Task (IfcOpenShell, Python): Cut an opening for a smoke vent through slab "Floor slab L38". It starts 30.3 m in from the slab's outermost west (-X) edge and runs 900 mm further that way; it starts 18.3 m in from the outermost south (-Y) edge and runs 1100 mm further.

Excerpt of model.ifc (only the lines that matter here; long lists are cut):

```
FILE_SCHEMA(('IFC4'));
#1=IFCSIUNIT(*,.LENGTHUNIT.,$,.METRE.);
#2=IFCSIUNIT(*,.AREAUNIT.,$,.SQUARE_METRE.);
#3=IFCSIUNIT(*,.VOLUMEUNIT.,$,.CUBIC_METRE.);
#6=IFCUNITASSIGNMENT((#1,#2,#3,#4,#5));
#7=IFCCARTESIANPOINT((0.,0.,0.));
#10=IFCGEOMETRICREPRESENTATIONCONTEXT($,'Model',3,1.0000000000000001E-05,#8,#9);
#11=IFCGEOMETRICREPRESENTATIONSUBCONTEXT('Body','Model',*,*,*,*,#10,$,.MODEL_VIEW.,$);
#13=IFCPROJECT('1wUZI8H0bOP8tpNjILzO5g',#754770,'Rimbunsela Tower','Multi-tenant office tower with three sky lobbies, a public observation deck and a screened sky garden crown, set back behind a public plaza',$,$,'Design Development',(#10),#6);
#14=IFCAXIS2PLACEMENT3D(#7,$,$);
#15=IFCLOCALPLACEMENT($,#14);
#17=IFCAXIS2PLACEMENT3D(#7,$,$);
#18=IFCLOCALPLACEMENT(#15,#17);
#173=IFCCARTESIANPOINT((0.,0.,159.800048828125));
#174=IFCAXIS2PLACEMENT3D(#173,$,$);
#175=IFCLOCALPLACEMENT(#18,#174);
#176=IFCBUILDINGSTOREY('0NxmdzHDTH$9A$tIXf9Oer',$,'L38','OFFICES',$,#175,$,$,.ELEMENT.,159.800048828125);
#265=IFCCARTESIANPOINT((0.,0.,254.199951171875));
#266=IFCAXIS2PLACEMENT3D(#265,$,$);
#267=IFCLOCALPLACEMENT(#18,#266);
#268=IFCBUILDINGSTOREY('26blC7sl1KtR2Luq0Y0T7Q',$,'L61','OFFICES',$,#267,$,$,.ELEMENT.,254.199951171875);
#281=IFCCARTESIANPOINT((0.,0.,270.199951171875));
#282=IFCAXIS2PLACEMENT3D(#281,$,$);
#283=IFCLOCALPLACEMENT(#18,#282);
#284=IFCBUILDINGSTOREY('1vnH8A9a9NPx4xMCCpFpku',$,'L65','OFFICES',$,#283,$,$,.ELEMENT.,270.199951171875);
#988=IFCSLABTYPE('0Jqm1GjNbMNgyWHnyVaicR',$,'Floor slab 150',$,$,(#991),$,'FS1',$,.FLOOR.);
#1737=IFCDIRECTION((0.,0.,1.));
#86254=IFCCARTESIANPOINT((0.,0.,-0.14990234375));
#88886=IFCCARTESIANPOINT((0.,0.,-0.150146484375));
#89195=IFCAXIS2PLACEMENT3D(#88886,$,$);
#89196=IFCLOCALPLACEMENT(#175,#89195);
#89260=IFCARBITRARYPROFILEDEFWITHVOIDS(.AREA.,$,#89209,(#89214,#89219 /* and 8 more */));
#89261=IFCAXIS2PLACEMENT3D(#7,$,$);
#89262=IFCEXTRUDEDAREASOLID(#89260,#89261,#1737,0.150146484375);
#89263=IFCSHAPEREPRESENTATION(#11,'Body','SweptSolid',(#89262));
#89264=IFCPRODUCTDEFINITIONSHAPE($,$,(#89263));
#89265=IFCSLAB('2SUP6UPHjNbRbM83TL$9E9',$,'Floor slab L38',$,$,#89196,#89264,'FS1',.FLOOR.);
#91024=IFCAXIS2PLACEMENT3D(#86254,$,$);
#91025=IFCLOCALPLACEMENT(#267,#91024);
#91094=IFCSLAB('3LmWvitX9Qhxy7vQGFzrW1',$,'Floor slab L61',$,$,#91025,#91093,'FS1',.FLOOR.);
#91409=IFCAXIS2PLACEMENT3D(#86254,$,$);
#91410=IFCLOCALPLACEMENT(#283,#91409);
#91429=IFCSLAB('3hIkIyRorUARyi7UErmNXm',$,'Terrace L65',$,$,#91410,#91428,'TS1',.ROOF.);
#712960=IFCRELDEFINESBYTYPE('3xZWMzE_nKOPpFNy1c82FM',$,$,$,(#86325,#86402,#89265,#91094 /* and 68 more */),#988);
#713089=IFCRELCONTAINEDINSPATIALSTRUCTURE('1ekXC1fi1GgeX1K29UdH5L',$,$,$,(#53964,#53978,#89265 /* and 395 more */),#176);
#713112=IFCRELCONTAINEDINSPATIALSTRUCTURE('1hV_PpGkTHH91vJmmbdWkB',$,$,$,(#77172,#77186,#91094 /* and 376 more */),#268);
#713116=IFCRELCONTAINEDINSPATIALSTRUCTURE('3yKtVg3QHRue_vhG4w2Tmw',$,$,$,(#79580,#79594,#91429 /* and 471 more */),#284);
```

```python
import numpy as np
import ifcopenshell
import ifcopenshell.api.feature
import ifcopenshell.api.geometry
import ifcopenshell.api.root
import ifcopenshell.geom
import ifcopenshell.util.placement
import ifcopenshell.util.representation
import ifcopenshell.util.shape
import ifcopenshell.util.unit

model = ifcopenshell.open("model.ifc")
unit_scale = ifcopenshell.util.unit.calculate_unit_scale(model)
settings = ifcopenshell.geom.settings()


def volume(element):
    """Net volume in cubic metres, openings subtracted."""
    shape = ifcopenshell.geom.create_shape(settings, element)
    return ifcopenshell.util.shape.get_volume(shape.geometry)


slab = model.by_guid("2SUP6UPHjNbRbM83TL$9E9")
before = volume(slab)

# Extent in the slab's own axes, in metres. The edges named are its -X and -Y sides.
slab_shape = ifcopenshell.geom.create_shape(settings, slab)
vertices = ifcopenshell.util.shape.get_vertices(slab_shape.geometry)
x_min, y_min, bottom = vertices.min(axis=0)
top = vertices[:, 2].max()

opening = ifcopenshell.api.root.create_entity(model, ifc_class="IfcOpeningElement", name="Smoke vent opening", predefined_type="OPENING")
context = ifcopenshell.util.representation.get_context(model, "Model", "Body", "MODEL_VIEW")
width, depth = 0.9, 1.1
outline = [(0.0, 0.0), (width, 0.0), (width, depth), (0.0, depth), (0.0, 0.0)]
# Overshoot both faces by 50 mm so the cut is clean.
shape = ifcopenshell.api.geometry.add_slab_representation(
    model, context=context, depth=top - bottom + 0.1, polyline=outline
)
ifcopenshell.api.geometry.assign_representation(model, product=opening, representation=shape)

matrix = ifcopenshell.util.placement.get_local_placement(slab.ObjectPlacement)
matrix[:, 3] = matrix @ np.append(np.array([x_min + 30.3, y_min + 18.3, bottom - 0.05]) / unit_scale, 1.0)
ifcopenshell.api.geometry.edit_object_placement(model, product=opening, matrix=matrix, is_si=False)
ifcopenshell.api.feature.add_feature(model, feature=opening, element=slab)

after = volume(slab)

print(f"slab volume {before:.3f} -> {after:.3f} m3")

model.write("model_v2.ifc")
```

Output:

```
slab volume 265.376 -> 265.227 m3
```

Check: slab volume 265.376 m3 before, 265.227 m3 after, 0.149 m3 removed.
